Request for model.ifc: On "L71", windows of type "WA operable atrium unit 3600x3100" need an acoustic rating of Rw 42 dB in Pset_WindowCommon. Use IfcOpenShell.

First a look at what the model holds.

```python
import ifcopenshell
import ifcopenshell.util.element

model = ifcopenshell.open("model.ifc")
print(model.schema)
storey = next(s for s in model.by_type("IfcBuildingStorey") if s.Name == "L71")
windows = [e for e in ifcopenshell.util.element.get_decomposition(storey) if e.is_a("IfcWindow")]
seen = {}
for e in windows:
    element_type = ifcopenshell.util.element.get_type(e)
    key = (element_type.Name if element_type != e and element_type else None, ifcopenshell.util.element.get_pset(e, "Pset_WindowCommon", "AcousticRating"))
    seen[key] = seen.get(key, 0) + 1
for (name, value), count in sorted(seen.items(), key=str):
    print(count, "x", name, "|", value)
```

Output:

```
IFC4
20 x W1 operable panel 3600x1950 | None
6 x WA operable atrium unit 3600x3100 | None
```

```python
import ifcopenshell
import ifcopenshell.api.pset
import ifcopenshell.util.element

model = ifcopenshell.open("model.ifc")

storey = next(s for s in model.by_type("IfcBuildingStorey") if s.Name == "L71")
windows = [e for e in ifcopenshell.util.element.get_decomposition(storey) if e.is_a("IfcWindow")]

count = 0
for e in windows:
    element_type = ifcopenshell.util.element.get_type(e)
    if element_type in (None, e) or element_type.Name != "WA operable atrium unit 3600x3100":
        continue
    found = ifcopenshell.util.element.get_pset(e, "Pset_WindowCommon", should_inherit=False)
    if found:
        pset = model.by_id(found["id"])
        if len(ifcopenshell.util.element.get_elements_by_pset(pset)) > 1:
            pset = ifcopenshell.api.pset.unshare_pset(model, products=[e], pset=pset)[0]
    else:
        pset = ifcopenshell.api.pset.add_pset(model, product=e, name="Pset_WindowCommon")
    ifcopenshell.api.pset.edit_pset(model, pset=pset, properties={"AcousticRating": "Rw 42 dB"})
    count += 1

print(count, "windows updated")

model.write("model_rev.ifc")
```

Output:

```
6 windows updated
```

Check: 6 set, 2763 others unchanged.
